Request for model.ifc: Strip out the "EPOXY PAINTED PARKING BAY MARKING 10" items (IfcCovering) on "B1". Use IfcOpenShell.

First a look at what the model holds.

```python
import ifcopenshell
import ifcopenshell.util.element

model = ifcopenshell.open("model.ifc")
print(model.schema)
storey = next(s for s in model.by_type("IfcBuildingStorey") if s.Name == "B1")
coverings = [e for e in ifcopenshell.util.element.get_decomposition(storey) if e.is_a("IfcCovering")]
seen = {}
for e in coverings:
    element_type = ifcopenshell.util.element.get_type(e)
    name = element_type.Name if element_type not in (None, e) else None
    seen[name] = seen.get(name, 0) + 1
for name, count in sorted(seen.items(), key=str):
    print(count, "x", name)
```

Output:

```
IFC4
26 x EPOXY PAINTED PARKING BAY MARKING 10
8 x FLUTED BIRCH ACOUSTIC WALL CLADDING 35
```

```python
import ifcopenshell
import ifcopenshell.api.root
import ifcopenshell.util.element

model = ifcopenshell.open("model.ifc")

storey = next(s for s in model.by_type("IfcBuildingStorey") if s.Name == "B1")
coverings = [e for e in ifcopenshell.util.element.get_decomposition(storey) if e.is_a("IfcCovering")]
targets = [e for e in coverings if (t := ifcopenshell.util.element.get_type(e)) not in (None, e) and t.Name == "EPOXY PAINTED PARKING BAY MARKING 10"]

for e in targets:
    ifcopenshell.api.root.remove_product(model, product=e)
print(len(targets), "removed")

model.write("model_v2.ifc")
```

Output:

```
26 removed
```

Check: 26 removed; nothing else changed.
